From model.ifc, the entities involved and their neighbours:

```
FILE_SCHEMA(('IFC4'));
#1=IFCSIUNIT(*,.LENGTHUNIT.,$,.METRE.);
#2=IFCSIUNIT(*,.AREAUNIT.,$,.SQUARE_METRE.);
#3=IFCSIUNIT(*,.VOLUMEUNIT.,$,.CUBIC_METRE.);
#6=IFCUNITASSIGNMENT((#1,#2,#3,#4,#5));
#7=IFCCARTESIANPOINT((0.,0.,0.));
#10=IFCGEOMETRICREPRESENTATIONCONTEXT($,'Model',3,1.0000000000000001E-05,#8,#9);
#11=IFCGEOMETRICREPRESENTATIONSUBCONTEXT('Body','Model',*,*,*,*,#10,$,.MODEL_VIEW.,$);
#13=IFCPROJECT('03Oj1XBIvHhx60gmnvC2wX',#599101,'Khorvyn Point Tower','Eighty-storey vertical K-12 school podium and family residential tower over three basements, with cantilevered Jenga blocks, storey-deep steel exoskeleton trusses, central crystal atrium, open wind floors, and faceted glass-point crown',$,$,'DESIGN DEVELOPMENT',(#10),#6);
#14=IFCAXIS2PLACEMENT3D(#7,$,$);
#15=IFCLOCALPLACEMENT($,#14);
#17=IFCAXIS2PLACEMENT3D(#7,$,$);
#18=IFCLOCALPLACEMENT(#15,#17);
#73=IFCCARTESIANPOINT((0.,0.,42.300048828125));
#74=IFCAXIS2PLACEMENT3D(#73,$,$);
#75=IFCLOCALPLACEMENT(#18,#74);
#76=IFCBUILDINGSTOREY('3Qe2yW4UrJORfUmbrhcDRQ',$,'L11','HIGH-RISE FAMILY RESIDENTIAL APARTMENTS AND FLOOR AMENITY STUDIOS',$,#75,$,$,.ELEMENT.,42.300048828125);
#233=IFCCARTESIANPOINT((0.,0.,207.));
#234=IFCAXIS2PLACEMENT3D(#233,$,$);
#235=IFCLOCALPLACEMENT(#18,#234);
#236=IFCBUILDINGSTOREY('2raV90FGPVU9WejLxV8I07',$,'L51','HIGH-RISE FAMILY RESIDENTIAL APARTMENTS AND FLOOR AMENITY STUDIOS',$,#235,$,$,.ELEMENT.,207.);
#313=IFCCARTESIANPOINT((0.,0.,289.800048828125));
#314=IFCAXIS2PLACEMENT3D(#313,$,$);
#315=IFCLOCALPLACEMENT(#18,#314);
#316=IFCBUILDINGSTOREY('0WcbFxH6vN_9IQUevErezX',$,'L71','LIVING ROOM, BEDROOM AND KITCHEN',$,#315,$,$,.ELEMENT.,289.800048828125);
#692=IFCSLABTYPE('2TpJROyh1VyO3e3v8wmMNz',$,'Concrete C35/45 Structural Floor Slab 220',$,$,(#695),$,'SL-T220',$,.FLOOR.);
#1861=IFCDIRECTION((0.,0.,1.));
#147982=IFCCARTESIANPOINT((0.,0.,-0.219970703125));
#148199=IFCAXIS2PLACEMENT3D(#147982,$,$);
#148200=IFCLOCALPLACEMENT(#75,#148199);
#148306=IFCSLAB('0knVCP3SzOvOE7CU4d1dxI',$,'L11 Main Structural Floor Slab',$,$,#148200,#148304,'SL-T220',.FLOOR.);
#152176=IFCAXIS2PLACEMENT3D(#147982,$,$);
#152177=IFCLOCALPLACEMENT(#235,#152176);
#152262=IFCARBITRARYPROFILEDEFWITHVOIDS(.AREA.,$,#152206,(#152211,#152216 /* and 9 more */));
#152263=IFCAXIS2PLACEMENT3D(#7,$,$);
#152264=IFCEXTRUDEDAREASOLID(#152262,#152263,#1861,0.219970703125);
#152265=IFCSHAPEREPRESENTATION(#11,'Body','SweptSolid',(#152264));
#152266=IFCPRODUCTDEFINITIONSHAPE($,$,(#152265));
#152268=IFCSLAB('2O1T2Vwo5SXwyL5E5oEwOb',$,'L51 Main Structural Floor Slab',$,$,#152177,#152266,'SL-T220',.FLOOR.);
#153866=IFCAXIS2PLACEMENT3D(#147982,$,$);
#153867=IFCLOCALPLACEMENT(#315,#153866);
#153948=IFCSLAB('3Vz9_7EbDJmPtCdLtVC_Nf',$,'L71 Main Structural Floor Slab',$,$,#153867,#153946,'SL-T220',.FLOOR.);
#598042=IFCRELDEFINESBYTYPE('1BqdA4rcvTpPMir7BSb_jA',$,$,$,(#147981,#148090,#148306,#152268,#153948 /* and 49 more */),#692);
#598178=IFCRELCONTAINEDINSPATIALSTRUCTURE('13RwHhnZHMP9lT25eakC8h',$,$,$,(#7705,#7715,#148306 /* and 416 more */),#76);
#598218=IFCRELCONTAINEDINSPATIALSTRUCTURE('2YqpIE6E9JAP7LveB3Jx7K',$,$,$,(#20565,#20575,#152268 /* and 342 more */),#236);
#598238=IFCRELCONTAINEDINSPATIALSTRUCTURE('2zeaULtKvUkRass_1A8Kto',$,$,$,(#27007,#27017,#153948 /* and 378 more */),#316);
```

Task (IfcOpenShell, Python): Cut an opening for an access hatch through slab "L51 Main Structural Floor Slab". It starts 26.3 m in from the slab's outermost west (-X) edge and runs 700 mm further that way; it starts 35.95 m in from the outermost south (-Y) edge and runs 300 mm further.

```python
import numpy as np
import ifcopenshell
import ifcopenshell.api.feature
import ifcopenshell.api.geometry
import ifcopenshell.api.root
import ifcopenshell.geom
import ifcopenshell.util.placement
import ifcopenshell.util.representation
import ifcopenshell.util.shape
import ifcopenshell.util.unit

model = ifcopenshell.open("model.ifc")
unit_scale = ifcopenshell.util.unit.calculate_unit_scale(model)
settings = ifcopenshell.geom.settings()


def volume(element):
    """Net volume in cubic metres, openings subtracted."""
    shape = ifcopenshell.geom.create_shape(settings, element)
    return ifcopenshell.util.shape.get_volume(shape.geometry)


slab = model.by_id(152268)
before = volume(slab)

# Extent in the slab's own axes, in metres. The edges named are its -X and -Y sides.
slab_shape = ifcopenshell.geom.create_shape(settings, slab)
vertices = ifcopenshell.util.shape.get_vertices(slab_shape.geometry)
x_min, y_min, bottom = vertices.min(axis=0)
top = vertices[:, 2].max()

opening = ifcopenshell.api.root.create_entity(model, ifc_class="IfcOpeningElement", name="Access hatch opening", predefined_type="OPENING")
context = ifcopenshell.util.representation.get_context(model, "Model", "Body", "MODEL_VIEW")
width, depth = 0.7, 0.3
outline = [(0.0, 0.0), (width, 0.0), (width, depth), (0.0, depth), (0.0, 0.0)]
# Overshoot both faces by 50 mm so the cut is clean.
shape = ifcopenshell.api.geometry.add_slab_representation(
    model, context=context, depth=top - bottom + 0.1, polyline=outline
)
ifcopenshell.api.geometry.assign_representation(model, product=opening, representation=shape)

matrix = ifcopenshell.util.placement.get_local_placement(slab.ObjectPlacement)
matrix[:, 3] = matrix @ np.append(np.array([x_min + 26.3, y_min + 35.95, bottom - 0.05]) / unit_scale, 1.0)
ifcopenshell.api.geometry.edit_object_placement(model, product=opening, matrix=matrix, is_si=False)
ifcopenshell.api.feature.add_feature(model, feature=opening, element=slab)

after = volume(slab)

print(f"slab volume {before:.3f} -> {after:.3f} m3")

model.write("model_edited.ifc")
```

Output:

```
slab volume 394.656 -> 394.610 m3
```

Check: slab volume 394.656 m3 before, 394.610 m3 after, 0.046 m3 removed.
